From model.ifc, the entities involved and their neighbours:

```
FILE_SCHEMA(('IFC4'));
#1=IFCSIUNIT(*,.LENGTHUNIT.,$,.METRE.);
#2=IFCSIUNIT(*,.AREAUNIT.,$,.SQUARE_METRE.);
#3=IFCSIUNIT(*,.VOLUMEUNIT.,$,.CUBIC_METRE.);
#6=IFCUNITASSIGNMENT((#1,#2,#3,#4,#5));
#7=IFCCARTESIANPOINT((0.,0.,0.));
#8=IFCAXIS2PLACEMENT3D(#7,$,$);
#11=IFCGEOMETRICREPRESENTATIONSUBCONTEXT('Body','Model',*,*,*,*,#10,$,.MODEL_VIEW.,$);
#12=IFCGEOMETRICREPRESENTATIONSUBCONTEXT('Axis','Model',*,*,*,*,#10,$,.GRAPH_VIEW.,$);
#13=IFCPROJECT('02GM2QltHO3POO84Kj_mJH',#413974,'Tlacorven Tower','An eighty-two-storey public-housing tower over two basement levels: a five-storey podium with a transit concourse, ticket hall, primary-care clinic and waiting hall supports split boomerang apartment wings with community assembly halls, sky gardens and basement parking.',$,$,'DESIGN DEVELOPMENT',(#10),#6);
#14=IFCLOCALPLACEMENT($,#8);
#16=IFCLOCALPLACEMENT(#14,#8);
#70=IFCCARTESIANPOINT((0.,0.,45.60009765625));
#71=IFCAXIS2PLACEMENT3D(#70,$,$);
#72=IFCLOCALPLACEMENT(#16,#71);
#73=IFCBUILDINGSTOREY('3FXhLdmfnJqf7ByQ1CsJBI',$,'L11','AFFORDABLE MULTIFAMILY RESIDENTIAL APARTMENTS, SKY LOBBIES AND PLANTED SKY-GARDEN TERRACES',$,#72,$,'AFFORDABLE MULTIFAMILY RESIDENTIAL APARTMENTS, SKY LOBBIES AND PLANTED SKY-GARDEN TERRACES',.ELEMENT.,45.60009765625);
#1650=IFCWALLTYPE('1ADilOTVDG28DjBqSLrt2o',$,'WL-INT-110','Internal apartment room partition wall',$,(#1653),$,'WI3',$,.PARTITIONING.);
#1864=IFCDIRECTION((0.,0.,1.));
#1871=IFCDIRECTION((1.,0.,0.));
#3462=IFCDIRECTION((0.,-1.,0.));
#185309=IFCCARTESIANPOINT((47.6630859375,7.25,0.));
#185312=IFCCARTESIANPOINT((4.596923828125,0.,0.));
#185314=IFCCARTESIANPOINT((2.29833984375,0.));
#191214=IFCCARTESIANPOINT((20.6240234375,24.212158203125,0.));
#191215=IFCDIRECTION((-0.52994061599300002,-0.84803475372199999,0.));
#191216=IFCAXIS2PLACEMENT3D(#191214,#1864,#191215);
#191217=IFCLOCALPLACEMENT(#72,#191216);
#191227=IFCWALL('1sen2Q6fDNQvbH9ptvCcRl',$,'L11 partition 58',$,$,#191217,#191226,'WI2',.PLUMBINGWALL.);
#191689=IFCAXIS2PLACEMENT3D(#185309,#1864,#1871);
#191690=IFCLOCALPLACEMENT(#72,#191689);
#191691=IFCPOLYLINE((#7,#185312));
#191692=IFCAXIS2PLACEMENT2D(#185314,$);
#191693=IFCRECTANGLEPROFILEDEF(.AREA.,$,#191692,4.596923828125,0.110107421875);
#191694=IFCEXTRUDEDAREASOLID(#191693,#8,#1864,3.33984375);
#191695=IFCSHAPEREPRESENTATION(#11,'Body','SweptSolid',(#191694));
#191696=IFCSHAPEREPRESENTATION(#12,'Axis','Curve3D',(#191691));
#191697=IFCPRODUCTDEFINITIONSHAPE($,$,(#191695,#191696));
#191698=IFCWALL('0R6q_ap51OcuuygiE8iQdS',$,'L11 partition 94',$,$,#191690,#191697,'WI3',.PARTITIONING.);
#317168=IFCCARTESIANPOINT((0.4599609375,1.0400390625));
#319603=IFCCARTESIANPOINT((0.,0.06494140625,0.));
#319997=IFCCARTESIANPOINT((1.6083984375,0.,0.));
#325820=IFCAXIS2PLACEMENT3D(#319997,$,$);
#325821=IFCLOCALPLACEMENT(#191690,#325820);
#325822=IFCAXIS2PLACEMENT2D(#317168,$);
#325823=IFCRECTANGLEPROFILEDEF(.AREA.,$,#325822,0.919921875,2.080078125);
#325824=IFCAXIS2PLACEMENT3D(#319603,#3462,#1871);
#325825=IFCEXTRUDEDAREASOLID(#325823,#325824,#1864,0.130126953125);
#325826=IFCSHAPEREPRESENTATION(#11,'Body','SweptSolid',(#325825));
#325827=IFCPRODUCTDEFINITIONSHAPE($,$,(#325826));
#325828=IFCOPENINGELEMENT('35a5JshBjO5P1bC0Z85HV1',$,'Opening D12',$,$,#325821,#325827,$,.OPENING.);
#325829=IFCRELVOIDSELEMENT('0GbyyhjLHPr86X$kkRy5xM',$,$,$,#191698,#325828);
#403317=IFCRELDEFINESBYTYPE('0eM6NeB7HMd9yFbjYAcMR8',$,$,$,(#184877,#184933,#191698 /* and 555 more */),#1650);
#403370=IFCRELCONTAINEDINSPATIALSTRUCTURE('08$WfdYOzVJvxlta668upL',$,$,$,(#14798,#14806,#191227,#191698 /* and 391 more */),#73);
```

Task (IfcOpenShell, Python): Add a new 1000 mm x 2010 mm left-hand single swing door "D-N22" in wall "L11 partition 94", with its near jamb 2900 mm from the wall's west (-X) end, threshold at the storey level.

```python
import numpy as np
import ifcopenshell
import ifcopenshell.api.feature
import ifcopenshell.api.geometry
import ifcopenshell.api.root
import ifcopenshell.api.spatial
import ifcopenshell.geom
import ifcopenshell.util.element
import ifcopenshell.util.placement
import ifcopenshell.util.representation
import ifcopenshell.util.shape
import ifcopenshell.util.unit

model = ifcopenshell.open("model.ifc")
unit_scale = ifcopenshell.util.unit.calculate_unit_scale(model)
settings = ifcopenshell.geom.settings()


def volume(element):
    """Net volume in cubic metres, openings subtracted."""
    shape = ifcopenshell.geom.create_shape(settings, element)
    return ifcopenshell.util.shape.get_volume(shape.geometry)


wall = model.by_guid("0R6q_ap51OcuuygiE8iQdS")
storey = ifcopenshell.util.element.get_container(wall, ifc_class="IfcBuildingStorey")
context = ifcopenshell.util.representation.get_context(model, "Model", "Body", "MODEL_VIEW")
before = volume(wall)

width, height, from_end, sill = 1, 2.01, 2.9, 0.0  # metres

# The wall runs along its own X axis, and the end named is its -X end.
wall_shape = ifcopenshell.geom.create_shape(settings, wall)
x, y, z = ifcopenshell.util.shape.get_vertices(wall_shape.geometry).T
start = x.min() + from_end
face, thickness = float(y.min()), float(y.max() - y.min())
wall_matrix = ifcopenshell.util.placement.get_local_placement(wall.ObjectPlacement)
level = ifcopenshell.util.placement.get_local_placement(storey.ObjectPlacement)[2, 3]


def in_wall(x, y):
    """Placement at x, y metres in the wall's axes, at sill height."""
    matrix = wall_matrix.copy()
    matrix[:, 3] = wall_matrix @ np.array([x / unit_scale, y / unit_scale, 0.0, 1.0])
    matrix[2, 3] = level + sill / unit_scale
    return matrix


# Opening: a box that overshoots both wall faces by 50 mm.
opening = ifcopenshell.api.root.create_entity(model, ifc_class="IfcOpeningElement", predefined_type="OPENING")
box = ifcopenshell.api.geometry.add_wall_representation(
    model, context=context, length=width, height=height, thickness=thickness + 0.1
)
ifcopenshell.api.geometry.assign_representation(model, product=opening, representation=box)
ifcopenshell.api.geometry.edit_object_placement(model, product=opening, matrix=in_wall(start, face - 0.05), is_si=False)
ifcopenshell.api.feature.add_feature(model, feature=opening, element=wall)

door = ifcopenshell.api.root.create_entity(model, ifc_class="IfcDoor", name="D-N22", predefined_type="DOOR")
door.OverallWidth, door.OverallHeight = width / unit_scale, height / unit_scale
door.OperationType = "SINGLE_SWING_LEFT"
body = ifcopenshell.api.geometry.add_door_representation(
    model,
    context=context,
    overall_width=door.OverallWidth,
    overall_height=door.OverallHeight,
    operation_type="SINGLE_SWING_LEFT",
    lining_properties={"LiningDepth": thickness / unit_scale, "ThresholdDepth": thickness / unit_scale},
)
ifcopenshell.api.geometry.assign_representation(model, product=door, representation=body)
ifcopenshell.api.spatial.assign_container(model, products=[door], relating_structure=storey)
ifcopenshell.api.feature.add_filling(model, opening=opening, element=door)

# The lining spans the wall, so the door starts at the wall face.
ifcopenshell.api.geometry.edit_object_placement(model, product=door, matrix=in_wall(start, face), is_si=False)

after = volume(wall)

print(f"wall volume {before:.3f} -> {after:.3f} m3")

model.write("model_updated.ifc")
```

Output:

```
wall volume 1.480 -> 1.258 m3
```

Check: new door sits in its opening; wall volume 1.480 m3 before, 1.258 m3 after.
